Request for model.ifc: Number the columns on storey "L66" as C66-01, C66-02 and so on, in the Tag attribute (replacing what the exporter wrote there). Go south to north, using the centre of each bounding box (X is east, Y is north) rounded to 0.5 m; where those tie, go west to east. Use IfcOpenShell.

First a look at what the model holds.

```python
import ifcopenshell
import ifcopenshell.util.element
import ifcopenshell.util.placement

model = ifcopenshell.open("model.ifc")
print(model.schema)
storey = next(s for s in model.by_type("IfcBuildingStorey") if s.Name == "L66")
columns = [e for e in ifcopenshell.util.element.get_decomposition(storey) if e.is_a("IfcColumn")]
for e in sorted(columns, key=lambda e: e.id()):
    origin = ifcopenshell.util.placement.get_local_placement(e.ObjectPlacement)[:3, 3]
    print(e.id(), e.Tag, e.Name, origin.round(2) + 0.0, sep=" | ")
```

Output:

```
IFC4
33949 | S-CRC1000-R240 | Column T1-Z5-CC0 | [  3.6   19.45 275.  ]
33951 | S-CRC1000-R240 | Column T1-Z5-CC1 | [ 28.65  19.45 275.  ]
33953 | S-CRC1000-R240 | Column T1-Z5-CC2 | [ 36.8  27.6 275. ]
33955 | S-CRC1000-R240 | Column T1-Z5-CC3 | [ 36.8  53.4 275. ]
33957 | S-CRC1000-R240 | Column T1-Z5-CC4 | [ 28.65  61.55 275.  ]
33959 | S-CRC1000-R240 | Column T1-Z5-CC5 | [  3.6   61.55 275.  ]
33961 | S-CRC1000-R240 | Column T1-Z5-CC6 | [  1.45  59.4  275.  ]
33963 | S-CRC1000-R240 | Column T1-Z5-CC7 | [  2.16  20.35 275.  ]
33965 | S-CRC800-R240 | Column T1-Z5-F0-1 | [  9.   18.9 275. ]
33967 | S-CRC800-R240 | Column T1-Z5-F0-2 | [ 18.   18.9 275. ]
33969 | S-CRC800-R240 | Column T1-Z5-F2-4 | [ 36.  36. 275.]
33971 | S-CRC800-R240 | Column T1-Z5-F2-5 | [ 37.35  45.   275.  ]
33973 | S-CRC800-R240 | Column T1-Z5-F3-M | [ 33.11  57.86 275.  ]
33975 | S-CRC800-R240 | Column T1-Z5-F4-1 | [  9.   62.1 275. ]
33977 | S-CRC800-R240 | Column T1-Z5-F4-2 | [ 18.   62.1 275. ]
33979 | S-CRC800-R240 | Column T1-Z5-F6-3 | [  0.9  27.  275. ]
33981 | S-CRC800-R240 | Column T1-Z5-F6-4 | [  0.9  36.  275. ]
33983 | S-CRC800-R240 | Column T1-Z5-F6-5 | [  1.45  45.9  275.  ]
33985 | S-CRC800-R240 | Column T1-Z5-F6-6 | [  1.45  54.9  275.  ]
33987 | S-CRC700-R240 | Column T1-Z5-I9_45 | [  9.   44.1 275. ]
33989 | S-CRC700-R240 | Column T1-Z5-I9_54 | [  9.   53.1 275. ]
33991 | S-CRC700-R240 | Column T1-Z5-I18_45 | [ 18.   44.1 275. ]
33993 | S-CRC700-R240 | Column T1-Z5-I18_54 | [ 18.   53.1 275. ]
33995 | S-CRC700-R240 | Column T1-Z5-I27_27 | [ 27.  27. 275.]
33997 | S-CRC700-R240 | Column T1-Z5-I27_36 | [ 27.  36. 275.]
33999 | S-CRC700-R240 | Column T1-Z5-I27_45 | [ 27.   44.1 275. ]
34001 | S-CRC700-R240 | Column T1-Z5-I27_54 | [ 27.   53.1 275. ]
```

```python
import ifcopenshell
import ifcopenshell.geom
import ifcopenshell.util.element
import ifcopenshell.util.shape

model = ifcopenshell.open("model.ifc")
settings = ifcopenshell.geom.settings()
settings.set("use-world-coords", True)


def centre(element):
    shape = ifcopenshell.geom.create_shape(settings, element)
    return ifcopenshell.util.shape.get_bbox_centroid(shape.geometry)


storey = next(s for s in model.by_type("IfcBuildingStorey") if s.Name == "L66")
columns = [e for e in ifcopenshell.util.element.get_decomposition(storey) if e.is_a("IfcColumn")]

# Insertion points can sit at a corner or the storey origin, so sort by the geometry (in metres).
centres = {e: centre(e) for e in columns}
columns.sort(key=lambda e: (round(centres[e][1] / 0.5), centres[e][0]))

for i, e in enumerate(columns, start=1):
    number = f"C66-{i:02d}"
    e.Tag = number
    print(e.id(), number)

model.write("model-out.ifc")
```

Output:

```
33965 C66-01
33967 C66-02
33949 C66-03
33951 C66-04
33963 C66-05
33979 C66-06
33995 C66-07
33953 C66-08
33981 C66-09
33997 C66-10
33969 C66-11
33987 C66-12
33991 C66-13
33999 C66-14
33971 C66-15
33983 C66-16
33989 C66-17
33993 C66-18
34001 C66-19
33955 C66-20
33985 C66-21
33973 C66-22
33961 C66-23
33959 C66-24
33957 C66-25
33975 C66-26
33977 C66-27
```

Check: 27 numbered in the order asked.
